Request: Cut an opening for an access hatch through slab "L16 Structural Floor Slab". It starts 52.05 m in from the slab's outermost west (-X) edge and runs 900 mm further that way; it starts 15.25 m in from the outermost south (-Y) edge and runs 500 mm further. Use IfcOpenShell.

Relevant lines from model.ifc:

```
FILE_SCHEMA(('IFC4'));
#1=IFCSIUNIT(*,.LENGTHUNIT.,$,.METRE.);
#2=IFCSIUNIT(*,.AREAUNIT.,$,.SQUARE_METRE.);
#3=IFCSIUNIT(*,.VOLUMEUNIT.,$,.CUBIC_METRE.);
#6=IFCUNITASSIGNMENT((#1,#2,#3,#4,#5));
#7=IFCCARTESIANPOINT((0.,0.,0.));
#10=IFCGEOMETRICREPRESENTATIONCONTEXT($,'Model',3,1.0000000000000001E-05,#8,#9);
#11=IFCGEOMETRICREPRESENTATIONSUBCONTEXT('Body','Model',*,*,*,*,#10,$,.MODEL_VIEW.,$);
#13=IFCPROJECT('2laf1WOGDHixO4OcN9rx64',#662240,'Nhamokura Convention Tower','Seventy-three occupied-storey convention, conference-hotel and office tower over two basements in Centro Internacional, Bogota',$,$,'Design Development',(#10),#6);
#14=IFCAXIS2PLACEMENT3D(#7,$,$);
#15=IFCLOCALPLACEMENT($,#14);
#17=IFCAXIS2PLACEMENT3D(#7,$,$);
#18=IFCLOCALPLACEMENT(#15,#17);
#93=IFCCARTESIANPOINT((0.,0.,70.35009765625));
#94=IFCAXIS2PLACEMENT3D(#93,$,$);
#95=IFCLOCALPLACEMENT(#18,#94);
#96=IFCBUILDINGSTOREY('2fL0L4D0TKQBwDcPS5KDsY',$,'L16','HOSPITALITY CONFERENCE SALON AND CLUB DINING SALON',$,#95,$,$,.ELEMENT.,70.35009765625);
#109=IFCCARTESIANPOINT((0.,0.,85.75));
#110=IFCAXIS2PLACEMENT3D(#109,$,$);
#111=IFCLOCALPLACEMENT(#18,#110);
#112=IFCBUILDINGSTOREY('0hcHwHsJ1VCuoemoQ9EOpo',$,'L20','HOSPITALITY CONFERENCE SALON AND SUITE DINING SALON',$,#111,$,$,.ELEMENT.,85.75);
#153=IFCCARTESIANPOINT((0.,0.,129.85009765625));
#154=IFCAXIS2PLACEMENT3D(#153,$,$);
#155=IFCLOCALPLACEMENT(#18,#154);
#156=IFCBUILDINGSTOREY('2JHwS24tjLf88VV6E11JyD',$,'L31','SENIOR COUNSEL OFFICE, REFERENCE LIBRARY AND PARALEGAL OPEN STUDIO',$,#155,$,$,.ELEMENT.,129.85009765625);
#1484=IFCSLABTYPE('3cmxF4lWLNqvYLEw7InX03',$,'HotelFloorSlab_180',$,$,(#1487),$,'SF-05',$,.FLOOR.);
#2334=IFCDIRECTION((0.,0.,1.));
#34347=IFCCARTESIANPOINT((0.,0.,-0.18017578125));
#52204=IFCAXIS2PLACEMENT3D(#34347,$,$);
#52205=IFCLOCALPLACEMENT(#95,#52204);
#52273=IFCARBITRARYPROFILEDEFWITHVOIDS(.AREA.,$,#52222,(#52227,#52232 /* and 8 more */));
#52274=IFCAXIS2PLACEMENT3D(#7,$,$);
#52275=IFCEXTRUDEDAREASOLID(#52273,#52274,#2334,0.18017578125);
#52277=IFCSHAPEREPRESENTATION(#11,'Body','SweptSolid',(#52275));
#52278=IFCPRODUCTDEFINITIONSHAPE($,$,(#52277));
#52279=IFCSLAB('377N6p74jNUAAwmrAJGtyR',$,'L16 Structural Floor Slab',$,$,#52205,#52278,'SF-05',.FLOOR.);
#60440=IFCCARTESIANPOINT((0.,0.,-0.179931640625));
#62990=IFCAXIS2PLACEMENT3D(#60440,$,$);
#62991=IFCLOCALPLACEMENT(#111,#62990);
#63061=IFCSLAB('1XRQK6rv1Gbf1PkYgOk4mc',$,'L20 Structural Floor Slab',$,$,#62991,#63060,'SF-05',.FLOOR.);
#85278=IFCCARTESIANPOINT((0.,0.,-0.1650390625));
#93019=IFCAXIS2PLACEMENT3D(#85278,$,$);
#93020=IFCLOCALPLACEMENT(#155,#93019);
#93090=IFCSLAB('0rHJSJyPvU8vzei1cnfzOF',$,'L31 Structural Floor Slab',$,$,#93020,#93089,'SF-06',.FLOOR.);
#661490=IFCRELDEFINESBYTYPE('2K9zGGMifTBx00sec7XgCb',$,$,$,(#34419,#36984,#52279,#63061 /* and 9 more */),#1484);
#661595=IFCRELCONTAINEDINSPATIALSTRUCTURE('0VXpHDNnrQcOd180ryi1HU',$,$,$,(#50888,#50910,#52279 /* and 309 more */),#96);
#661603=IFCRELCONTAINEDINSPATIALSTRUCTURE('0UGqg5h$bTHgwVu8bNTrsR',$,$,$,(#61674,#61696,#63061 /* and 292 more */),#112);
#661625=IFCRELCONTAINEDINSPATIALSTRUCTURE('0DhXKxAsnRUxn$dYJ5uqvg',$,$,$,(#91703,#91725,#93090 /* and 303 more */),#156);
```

```python
import numpy as np
import ifcopenshell
import ifcopenshell.api.feature
import ifcopenshell.api.geometry
import ifcopenshell.api.root
import ifcopenshell.geom
import ifcopenshell.util.placement
import ifcopenshell.util.representation
import ifcopenshell.util.shape
import ifcopenshell.util.unit

model = ifcopenshell.open("model.ifc")
unit_scale = ifcopenshell.util.unit.calculate_unit_scale(model)
settings = ifcopenshell.geom.settings()


def volume(element):
    """Net volume in cubic metres, openings subtracted."""
    shape = ifcopenshell.geom.create_shape(settings, element)
    return ifcopenshell.util.shape.get_volume(shape.geometry)


slab = model.by_guid("377N6p74jNUAAwmrAJGtyR")
before = volume(slab)

# Extent in the slab's own axes, in metres. The edges named are its -X and -Y sides.
slab_shape = ifcopenshell.geom.create_shape(settings, slab)
vertices = ifcopenshell.util.shape.get_vertices(slab_shape.geometry)
x_min, y_min, bottom = vertices.min(axis=0)
top = vertices[:, 2].max()

opening = ifcopenshell.api.root.create_entity(model, ifc_class="IfcOpeningElement", name="Access hatch opening", predefined_type="OPENING")
context = ifcopenshell.util.representation.get_context(model, "Model", "Body", "MODEL_VIEW")
width, depth = 0.9, 0.5
outline = [(0.0, 0.0), (width, 0.0), (width, depth), (0.0, depth), (0.0, 0.0)]
# Overshoot both faces by 50 mm so the cut is clean.
shape = ifcopenshell.api.geometry.add_slab_representation(
    model, context=context, depth=top - bottom + 0.1, polyline=outline
)
ifcopenshell.api.geometry.assign_representation(model, product=opening, representation=shape)

matrix = ifcopenshell.util.placement.get_local_placement(slab.ObjectPlacement)
matrix[:, 3] = matrix @ np.append(np.array([x_min + 52.05, y_min + 15.25, bottom - 0.05]) / unit_scale, 1.0)
ifcopenshell.api.geometry.edit_object_placement(model, product=opening, matrix=matrix, is_si=False)
ifcopenshell.api.feature.add_feature(model, feature=opening, element=slab)

after = volume(slab)

print(f"slab volume {before:.3f} -> {after:.3f} m3")

model.write("model_v2.ifc")
```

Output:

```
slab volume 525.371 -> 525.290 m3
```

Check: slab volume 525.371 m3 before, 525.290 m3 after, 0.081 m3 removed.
